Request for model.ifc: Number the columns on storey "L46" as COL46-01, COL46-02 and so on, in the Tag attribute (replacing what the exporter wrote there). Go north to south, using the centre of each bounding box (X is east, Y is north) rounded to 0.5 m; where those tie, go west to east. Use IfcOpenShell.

First a look at what the model holds.

```python
import ifcopenshell
import ifcopenshell.util.element
import ifcopenshell.util.placement

model = ifcopenshell.open("model.ifc")
print(model.schema)
storey = next(s for s in model.by_type("IfcBuildingStorey") if s.Name == "L46")
columns = [e for e in ifcopenshell.util.element.get_decomposition(storey) if e.is_a("IfcColumn")]
for e in sorted(columns, key=lambda e: e.id()):
    origin = ifcopenshell.util.placement.get_local_placement(e.ObjectPlacement)[:3, 3]
    print(e.id(), e.Tag, e.Name, origin.round(2) + 0.0, sep=" | ")
```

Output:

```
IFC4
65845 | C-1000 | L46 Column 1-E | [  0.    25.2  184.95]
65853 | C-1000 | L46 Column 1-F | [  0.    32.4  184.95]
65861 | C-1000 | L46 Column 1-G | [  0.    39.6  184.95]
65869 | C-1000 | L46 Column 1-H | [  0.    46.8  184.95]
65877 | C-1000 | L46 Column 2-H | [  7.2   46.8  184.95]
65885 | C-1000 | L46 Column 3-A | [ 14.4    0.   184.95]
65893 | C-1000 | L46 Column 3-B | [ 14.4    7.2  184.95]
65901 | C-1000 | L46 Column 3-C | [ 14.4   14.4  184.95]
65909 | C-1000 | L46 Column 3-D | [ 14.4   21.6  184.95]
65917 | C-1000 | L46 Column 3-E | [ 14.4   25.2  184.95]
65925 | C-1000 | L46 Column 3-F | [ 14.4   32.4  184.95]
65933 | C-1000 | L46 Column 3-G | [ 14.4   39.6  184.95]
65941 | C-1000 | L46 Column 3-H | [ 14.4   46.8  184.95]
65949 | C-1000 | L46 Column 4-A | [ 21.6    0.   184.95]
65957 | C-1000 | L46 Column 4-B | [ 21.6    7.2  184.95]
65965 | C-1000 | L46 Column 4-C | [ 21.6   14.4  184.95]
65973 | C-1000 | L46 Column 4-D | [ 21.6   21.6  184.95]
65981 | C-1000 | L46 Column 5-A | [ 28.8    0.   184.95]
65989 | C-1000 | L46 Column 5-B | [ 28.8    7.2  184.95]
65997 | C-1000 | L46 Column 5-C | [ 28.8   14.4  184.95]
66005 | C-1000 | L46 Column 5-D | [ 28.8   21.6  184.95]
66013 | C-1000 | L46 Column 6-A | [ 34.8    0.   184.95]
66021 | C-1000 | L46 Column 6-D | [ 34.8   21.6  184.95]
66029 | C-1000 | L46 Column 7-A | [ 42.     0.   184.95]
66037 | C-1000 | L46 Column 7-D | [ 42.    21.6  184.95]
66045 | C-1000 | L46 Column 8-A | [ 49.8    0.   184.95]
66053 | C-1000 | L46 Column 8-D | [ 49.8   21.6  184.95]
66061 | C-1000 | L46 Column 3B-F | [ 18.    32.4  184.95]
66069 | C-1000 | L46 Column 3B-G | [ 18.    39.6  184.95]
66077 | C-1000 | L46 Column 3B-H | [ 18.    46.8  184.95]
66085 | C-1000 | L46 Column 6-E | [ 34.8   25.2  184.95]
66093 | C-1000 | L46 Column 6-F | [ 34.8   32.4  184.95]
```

```python
import ifcopenshell
import ifcopenshell.geom
import ifcopenshell.util.element
import ifcopenshell.util.shape

model = ifcopenshell.open("model.ifc")
settings = ifcopenshell.geom.settings()
settings.set("use-world-coords", True)


def centre(element):
    shape = ifcopenshell.geom.create_shape(settings, element)
    return ifcopenshell.util.shape.get_bbox_centroid(shape.geometry)


storey = next(s for s in model.by_type("IfcBuildingStorey") if s.Name == "L46")
columns = [e for e in ifcopenshell.util.element.get_decomposition(storey) if e.is_a("IfcColumn")]

# Insertion points can sit at a corner or the storey origin, so sort by the geometry (in metres).
centres = {e: centre(e) for e in columns}
columns.sort(key=lambda e: (-round(centres[e][1] / 0.5), centres[e][0]))

for i, e in enumerate(columns, start=1):
    number = f"COL46-{i:02d}"
    e.Tag = number
    print(e.id(), number)

model.write("model-out.ifc")
```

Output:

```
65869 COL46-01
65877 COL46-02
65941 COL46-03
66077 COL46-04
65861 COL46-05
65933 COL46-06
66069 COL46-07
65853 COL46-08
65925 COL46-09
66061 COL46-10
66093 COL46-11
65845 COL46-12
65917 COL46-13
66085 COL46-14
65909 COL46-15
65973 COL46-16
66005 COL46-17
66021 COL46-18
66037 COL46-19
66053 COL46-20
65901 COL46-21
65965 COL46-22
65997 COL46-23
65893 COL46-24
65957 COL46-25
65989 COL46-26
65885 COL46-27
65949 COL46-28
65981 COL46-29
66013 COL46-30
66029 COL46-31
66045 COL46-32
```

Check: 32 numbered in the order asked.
